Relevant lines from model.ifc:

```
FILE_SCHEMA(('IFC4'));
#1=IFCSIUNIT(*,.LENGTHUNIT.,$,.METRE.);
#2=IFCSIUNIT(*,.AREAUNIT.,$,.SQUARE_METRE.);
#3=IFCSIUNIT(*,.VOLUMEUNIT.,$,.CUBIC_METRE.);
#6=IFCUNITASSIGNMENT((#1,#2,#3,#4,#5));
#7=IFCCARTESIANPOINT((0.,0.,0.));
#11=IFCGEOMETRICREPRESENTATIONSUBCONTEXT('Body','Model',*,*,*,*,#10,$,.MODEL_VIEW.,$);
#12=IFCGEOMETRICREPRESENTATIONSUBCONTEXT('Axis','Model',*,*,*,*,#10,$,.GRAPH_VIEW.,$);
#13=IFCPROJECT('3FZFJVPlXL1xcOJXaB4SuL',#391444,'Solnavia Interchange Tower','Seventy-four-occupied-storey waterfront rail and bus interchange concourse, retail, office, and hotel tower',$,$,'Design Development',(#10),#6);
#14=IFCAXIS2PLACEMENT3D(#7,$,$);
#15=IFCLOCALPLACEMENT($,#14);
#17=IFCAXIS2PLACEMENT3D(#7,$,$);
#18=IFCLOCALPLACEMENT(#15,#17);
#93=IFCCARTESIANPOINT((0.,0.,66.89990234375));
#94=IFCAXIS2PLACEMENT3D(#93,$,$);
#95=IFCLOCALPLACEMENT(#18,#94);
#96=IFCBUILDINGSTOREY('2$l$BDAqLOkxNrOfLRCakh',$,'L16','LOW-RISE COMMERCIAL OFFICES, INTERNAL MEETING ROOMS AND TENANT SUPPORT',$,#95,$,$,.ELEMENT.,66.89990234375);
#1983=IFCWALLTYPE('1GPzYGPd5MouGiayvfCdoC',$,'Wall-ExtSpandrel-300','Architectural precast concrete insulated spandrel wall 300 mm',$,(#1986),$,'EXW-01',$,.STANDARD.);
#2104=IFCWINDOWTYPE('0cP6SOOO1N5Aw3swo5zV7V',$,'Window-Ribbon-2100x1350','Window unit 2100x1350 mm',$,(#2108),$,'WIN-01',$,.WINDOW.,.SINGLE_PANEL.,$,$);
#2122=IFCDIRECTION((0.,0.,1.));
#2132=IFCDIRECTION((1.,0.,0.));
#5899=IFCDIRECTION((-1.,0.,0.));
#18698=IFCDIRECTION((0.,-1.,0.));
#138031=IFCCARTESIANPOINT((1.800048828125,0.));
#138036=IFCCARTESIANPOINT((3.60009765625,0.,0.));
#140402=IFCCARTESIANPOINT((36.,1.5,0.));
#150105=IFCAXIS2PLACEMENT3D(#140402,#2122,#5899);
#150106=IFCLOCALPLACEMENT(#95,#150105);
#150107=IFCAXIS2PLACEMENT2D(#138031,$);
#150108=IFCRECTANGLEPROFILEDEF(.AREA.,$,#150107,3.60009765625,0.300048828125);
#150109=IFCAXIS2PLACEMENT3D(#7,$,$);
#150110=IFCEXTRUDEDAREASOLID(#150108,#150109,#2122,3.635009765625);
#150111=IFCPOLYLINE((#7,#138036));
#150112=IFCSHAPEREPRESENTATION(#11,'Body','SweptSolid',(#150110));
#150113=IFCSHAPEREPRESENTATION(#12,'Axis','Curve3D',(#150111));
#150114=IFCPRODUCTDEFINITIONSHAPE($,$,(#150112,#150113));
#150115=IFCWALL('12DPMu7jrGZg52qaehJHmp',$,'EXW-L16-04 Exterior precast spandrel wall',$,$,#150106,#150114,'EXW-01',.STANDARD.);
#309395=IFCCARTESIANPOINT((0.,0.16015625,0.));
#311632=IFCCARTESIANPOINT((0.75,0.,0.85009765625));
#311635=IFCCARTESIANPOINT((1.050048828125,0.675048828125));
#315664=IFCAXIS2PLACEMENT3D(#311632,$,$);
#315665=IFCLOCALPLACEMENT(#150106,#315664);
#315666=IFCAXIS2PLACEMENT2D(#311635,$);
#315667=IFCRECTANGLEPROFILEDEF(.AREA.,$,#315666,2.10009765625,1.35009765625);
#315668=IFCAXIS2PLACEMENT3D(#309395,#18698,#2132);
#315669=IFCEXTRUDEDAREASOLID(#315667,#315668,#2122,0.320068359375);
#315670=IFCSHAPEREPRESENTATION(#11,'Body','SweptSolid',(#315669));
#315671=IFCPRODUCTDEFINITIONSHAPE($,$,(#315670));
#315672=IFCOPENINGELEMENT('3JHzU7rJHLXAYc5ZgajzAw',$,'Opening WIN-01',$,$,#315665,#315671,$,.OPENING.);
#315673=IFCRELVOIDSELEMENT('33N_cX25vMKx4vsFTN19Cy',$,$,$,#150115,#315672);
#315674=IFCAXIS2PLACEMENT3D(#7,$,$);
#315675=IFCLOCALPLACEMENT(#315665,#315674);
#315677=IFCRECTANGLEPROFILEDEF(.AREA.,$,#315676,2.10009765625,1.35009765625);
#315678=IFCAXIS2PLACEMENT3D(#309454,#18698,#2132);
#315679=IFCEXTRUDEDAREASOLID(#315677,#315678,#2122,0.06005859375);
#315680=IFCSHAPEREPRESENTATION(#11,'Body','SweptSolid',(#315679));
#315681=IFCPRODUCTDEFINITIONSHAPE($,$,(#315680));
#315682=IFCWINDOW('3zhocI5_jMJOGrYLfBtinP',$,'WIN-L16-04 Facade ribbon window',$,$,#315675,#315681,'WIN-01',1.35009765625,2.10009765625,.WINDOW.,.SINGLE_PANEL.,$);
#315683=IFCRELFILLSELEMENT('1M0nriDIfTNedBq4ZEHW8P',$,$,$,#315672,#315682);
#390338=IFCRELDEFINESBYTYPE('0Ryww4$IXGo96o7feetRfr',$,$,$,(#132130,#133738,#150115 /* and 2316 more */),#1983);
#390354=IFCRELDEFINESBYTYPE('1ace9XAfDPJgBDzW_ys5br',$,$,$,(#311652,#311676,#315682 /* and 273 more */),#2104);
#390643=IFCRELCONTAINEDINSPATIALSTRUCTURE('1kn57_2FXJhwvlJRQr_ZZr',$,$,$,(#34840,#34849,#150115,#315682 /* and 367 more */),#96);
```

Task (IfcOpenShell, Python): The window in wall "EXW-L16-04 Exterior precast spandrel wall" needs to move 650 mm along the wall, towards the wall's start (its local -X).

```python
import ifcopenshell
import ifcopenshell.api.geometry
import ifcopenshell.util.placement

model = ifcopenshell.open("model.ifc")

window = model.by_guid("3zhocI5_jMJOGrYLfBtinP")
opening = window.FillsVoids[0].RelatingOpeningElement
wall = opening.VoidsElements[0].RelatingBuildingElement

wall_matrix = ifcopenshell.util.placement.get_local_placement(wall.ObjectPlacement)
shift = wall_matrix[:3, 0] * -0.65
before = ifcopenshell.util.placement.get_local_placement(window.ObjectPlacement)[:3, 3].copy()

# The window is placed relative to its opening, so it follows when the opening moves.
matrix = ifcopenshell.util.placement.get_local_placement(opening.ObjectPlacement)
matrix[:3, 3] += shift
ifcopenshell.api.geometry.edit_object_placement(
    model, product=opening, matrix=matrix, is_si=False, should_transform_children=True
)

after = ifcopenshell.util.placement.get_local_placement(window.ObjectPlacement)[:3, 3]
print("window moved by", (after - before).round(3) + 0.0)

model.write("model-out.ifc")
```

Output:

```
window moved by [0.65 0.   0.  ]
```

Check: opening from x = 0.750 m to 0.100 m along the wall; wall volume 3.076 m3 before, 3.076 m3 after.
